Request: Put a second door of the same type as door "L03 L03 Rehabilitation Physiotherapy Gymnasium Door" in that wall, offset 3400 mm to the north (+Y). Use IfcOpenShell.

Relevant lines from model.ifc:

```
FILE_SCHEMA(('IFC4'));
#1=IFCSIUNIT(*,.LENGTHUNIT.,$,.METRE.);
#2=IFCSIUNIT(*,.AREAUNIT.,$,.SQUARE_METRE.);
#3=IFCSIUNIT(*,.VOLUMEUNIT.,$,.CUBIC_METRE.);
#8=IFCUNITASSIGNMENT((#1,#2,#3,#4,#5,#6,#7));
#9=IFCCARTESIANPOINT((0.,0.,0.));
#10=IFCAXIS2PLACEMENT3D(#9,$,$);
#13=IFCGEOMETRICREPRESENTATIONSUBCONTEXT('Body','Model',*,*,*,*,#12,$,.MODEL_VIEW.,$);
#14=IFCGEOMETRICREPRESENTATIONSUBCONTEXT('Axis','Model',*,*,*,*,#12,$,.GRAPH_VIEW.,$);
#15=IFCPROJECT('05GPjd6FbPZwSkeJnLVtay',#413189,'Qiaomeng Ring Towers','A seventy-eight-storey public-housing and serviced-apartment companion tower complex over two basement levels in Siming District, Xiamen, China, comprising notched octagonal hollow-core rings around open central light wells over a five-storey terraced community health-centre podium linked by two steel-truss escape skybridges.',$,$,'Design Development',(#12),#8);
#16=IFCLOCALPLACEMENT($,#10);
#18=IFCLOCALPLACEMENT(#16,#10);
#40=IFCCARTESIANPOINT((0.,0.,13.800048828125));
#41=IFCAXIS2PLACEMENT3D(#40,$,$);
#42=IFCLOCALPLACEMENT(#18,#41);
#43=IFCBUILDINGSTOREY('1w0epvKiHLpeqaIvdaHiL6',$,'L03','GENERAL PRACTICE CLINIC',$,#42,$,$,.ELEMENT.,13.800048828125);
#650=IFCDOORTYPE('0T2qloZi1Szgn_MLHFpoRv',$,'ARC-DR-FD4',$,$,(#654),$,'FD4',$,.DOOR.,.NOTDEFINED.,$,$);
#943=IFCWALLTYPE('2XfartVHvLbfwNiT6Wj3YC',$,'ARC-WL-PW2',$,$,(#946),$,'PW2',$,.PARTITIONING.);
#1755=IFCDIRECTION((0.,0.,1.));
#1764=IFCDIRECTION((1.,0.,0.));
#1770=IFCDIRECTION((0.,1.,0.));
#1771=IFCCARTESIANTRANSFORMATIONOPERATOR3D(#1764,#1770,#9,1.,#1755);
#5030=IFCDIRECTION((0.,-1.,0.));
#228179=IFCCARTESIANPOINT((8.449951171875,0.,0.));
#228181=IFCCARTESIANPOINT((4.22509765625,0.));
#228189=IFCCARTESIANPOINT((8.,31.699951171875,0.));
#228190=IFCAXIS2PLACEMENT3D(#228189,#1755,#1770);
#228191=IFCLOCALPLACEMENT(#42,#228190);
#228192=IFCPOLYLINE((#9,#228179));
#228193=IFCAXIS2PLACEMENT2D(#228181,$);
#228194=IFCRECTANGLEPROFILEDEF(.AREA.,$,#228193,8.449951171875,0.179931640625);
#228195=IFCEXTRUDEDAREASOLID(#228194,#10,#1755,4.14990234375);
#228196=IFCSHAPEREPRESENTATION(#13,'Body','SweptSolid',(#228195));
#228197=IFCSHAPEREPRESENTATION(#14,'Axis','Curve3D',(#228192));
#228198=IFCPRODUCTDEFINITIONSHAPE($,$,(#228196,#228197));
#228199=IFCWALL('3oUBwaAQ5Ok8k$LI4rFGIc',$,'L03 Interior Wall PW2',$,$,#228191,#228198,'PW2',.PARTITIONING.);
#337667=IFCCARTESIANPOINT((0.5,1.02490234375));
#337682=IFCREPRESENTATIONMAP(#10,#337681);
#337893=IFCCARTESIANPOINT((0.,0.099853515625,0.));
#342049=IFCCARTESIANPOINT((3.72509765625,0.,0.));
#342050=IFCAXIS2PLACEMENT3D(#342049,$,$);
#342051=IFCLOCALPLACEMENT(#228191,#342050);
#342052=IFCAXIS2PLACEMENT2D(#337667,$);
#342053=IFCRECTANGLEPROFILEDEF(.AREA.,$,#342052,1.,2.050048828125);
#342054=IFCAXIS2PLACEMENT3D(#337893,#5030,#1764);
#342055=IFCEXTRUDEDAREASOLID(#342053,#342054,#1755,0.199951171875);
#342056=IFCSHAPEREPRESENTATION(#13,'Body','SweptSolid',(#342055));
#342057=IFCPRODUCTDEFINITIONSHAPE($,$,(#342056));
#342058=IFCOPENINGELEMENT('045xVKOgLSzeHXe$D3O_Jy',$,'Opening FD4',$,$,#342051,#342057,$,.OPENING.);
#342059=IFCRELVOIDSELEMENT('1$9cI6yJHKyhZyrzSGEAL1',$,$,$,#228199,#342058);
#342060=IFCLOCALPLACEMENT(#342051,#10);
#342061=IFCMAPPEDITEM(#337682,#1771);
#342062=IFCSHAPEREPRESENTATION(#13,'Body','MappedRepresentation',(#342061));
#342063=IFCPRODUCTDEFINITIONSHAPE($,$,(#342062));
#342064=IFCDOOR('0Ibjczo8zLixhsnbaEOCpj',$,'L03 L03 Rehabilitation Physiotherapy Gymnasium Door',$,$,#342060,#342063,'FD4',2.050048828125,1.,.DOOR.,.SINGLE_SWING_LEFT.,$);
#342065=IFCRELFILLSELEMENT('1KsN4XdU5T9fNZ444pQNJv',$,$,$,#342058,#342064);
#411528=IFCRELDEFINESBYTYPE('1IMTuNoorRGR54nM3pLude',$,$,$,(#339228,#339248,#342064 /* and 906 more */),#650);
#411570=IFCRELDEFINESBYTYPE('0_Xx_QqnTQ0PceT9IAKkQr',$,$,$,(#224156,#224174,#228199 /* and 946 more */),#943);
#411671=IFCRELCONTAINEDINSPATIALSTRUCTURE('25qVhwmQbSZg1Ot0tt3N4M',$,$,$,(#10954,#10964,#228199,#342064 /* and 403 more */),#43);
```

```python
import ifcopenshell
import ifcopenshell.api.feature
import ifcopenshell.api.geometry
import ifcopenshell.api.root
import ifcopenshell.geom
import ifcopenshell.util.element
import ifcopenshell.util.placement
import ifcopenshell.util.shape
import ifcopenshell.util.unit

model = ifcopenshell.open("model.ifc")
unit_scale = ifcopenshell.util.unit.calculate_unit_scale(model)
settings = ifcopenshell.geom.settings()


def volume(element):
    """Net volume in cubic metres, openings subtracted."""
    shape = ifcopenshell.geom.create_shape(settings, element)
    return ifcopenshell.util.shape.get_volume(shape.geometry)


door = model.by_guid("0Ibjczo8zLixhsnbaEOCpj")
opening = door.FillsVoids[0].RelatingOpeningElement
wall = opening.VoidsElements[0].RelatingBuildingElement
before = volume(wall)
shift = ifcopenshell.util.placement.get_local_placement(wall.ObjectPlacement)[:3, 0] * 3.4 / unit_scale

# copy_class copies the void relationship, type, container and properties, but no geometry.
new_opening = ifcopenshell.api.root.copy_class(model, product=opening)
new_opening.Representation = ifcopenshell.util.element.copy_deep(
    model, opening.Representation, exclude=["IfcGeometricRepresentationContext", "IfcRepresentationMap"]
)
new_door = ifcopenshell.api.root.copy_class(model, product=door)
new_door.Representation = ifcopenshell.util.element.copy_deep(
    model, door.Representation, exclude=["IfcGeometricRepresentationContext", "IfcRepresentationMap"]
)
new_door.Tag = None
ifcopenshell.api.feature.add_filling(model, opening=new_opening, element=new_door)

for old, new in ((opening, new_opening), (door, new_door)):
    matrix = ifcopenshell.util.placement.get_local_placement(old.ObjectPlacement)
    matrix[:3, 3] += shift
    ifcopenshell.api.geometry.edit_object_placement(model, product=new, matrix=matrix, is_si=False)

after = volume(wall)

print(f"wall volume {before:.3f} -> {after:.3f} m3")

model.write("model_edited.ifc")
```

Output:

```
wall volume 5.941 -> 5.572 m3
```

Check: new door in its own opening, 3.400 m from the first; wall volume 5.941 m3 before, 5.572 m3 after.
